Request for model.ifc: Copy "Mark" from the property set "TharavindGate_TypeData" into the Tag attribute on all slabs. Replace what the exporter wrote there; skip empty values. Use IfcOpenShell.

First a look at what the model holds.

```python
import ifcopenshell
import ifcopenshell.util.element

model = ifcopenshell.open("model.ifc")
print(model.schema)
slabs = model.by_type("IfcSlab")
print(len(slabs), "slabs")
for e in slabs[:8]:
    source = ifcopenshell.util.element.get_pset(e, "TharavindGate_TypeData", "Mark")
    target = e.Tag
    print(e.id(), repr(source), repr(target), sep=" | ")
```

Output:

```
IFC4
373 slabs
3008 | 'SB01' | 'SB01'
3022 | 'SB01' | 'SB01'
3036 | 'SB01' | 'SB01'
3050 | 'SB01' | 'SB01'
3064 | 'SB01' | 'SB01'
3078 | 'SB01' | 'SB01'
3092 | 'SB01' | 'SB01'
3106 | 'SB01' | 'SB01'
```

```python
import ifcopenshell
import ifcopenshell.util.element

model = ifcopenshell.open("model.ifc")

count = 0
for e in model.by_type("IfcSlab"):
    value = ifcopenshell.util.element.get_pset(e, "TharavindGate_TypeData", "Mark")
    current = e.Tag
    if not value or not value.strip() or current == value:
        continue
    e.Tag = value
    count += 1

print(count, "slabs updated")

model.write("model_edited.ifc")
```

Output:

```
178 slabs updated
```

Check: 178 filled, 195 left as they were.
